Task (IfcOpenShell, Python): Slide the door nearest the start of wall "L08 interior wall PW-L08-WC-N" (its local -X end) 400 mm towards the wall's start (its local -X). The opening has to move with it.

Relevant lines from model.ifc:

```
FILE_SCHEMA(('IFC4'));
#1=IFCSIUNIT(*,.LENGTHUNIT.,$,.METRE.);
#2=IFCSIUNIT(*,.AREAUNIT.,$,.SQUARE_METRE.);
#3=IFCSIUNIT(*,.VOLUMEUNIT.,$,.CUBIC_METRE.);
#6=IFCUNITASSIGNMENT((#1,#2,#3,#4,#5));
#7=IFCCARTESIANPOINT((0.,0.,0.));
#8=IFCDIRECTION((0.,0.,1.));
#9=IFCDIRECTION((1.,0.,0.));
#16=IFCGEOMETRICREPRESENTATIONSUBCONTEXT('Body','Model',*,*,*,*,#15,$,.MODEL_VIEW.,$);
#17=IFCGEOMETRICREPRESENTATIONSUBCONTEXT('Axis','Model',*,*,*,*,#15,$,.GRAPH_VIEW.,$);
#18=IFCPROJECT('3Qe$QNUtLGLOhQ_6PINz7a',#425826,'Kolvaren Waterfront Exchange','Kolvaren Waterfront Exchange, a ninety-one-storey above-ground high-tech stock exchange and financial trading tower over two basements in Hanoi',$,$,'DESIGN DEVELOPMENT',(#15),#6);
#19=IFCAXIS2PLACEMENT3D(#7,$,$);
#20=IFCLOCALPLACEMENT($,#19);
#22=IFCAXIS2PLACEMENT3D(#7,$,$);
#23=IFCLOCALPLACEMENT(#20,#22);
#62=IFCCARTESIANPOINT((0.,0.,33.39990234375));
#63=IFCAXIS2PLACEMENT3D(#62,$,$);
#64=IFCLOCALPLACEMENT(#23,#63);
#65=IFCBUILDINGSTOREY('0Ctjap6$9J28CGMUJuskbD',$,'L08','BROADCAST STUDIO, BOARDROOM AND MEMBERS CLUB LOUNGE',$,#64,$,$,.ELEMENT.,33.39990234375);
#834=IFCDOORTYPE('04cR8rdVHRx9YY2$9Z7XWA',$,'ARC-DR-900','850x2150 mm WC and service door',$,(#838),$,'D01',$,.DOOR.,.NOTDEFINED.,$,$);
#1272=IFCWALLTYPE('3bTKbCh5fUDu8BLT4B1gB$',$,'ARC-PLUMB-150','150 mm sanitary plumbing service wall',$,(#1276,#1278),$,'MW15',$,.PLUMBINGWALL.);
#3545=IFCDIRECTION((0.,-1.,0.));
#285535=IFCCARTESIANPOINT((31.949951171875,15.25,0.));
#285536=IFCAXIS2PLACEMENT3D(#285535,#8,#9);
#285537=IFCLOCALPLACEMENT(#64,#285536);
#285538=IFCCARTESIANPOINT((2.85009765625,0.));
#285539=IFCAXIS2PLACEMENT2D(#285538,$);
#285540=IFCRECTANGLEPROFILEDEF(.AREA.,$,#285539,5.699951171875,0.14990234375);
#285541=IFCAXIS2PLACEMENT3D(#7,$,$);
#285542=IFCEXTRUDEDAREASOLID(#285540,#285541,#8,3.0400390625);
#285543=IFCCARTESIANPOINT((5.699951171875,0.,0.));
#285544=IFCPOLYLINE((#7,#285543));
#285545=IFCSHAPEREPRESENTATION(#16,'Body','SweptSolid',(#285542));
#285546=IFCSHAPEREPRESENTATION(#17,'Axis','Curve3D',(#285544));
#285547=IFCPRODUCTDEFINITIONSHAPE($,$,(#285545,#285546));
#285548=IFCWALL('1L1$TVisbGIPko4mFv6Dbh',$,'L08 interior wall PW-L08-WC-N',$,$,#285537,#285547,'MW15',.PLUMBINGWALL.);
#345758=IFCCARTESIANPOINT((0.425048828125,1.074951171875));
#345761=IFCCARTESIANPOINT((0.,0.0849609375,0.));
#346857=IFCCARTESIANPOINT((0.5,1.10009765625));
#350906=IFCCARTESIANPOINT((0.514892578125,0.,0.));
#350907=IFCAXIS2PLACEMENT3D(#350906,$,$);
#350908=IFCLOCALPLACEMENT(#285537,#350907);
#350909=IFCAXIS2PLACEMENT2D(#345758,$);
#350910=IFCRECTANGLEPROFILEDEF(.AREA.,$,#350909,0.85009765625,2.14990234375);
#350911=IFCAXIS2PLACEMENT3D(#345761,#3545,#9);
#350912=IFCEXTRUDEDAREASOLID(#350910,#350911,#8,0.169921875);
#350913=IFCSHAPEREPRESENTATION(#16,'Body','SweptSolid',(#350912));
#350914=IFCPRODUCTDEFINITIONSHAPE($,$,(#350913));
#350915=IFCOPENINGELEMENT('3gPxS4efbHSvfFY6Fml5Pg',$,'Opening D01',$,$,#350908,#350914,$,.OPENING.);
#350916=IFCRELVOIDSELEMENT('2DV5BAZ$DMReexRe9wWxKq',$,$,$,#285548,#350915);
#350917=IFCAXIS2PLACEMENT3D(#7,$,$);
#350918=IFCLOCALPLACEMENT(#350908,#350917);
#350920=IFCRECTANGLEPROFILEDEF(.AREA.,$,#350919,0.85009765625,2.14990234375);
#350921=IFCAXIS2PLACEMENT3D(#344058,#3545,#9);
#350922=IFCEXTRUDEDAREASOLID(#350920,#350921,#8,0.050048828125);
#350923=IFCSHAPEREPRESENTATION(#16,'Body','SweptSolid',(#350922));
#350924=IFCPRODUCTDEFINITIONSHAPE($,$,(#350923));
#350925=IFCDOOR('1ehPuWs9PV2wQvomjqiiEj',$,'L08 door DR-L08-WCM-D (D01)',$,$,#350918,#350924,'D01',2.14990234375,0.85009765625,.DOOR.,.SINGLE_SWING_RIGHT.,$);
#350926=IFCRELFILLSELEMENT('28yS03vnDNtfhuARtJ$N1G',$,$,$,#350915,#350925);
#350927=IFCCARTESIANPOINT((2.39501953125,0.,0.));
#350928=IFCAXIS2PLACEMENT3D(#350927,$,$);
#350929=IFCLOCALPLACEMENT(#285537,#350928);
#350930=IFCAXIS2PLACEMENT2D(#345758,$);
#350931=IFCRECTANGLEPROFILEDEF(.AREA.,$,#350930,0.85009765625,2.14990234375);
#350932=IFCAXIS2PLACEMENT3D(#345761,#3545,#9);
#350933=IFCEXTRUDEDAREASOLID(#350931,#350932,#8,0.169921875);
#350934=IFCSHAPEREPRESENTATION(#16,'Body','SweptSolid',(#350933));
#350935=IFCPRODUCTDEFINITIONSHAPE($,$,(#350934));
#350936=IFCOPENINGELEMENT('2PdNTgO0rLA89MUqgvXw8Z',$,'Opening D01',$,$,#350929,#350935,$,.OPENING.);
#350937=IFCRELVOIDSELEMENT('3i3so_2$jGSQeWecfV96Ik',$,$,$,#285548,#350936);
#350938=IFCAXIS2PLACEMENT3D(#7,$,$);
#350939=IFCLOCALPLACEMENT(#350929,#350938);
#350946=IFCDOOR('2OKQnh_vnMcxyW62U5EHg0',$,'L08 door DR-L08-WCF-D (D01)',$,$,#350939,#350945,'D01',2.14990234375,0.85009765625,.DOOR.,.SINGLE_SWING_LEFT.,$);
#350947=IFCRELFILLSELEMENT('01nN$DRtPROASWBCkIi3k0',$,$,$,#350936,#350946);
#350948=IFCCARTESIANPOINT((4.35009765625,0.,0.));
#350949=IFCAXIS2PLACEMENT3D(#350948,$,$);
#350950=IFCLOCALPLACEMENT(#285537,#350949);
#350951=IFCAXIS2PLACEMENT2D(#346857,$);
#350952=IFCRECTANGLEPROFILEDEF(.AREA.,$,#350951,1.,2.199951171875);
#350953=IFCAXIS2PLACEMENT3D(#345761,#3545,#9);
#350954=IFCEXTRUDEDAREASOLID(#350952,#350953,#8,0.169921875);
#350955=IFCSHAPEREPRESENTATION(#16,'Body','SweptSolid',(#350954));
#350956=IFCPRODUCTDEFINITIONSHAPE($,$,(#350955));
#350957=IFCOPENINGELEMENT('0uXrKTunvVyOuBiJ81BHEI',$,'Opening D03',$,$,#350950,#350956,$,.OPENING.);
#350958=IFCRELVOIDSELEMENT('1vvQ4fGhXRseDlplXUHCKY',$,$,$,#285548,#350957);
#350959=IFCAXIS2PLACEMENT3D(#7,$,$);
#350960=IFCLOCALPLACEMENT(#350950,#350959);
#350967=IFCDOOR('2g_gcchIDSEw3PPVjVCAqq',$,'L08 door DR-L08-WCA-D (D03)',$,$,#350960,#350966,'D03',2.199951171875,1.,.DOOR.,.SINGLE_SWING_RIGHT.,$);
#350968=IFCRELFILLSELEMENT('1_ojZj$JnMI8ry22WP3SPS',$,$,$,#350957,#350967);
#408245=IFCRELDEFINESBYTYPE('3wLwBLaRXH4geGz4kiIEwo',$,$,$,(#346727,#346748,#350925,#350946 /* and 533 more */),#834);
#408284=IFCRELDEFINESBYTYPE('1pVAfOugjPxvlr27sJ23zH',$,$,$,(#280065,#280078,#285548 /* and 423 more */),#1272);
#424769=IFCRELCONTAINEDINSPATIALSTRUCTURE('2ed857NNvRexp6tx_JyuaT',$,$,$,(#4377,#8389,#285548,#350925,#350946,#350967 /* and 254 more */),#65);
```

```python
import ifcopenshell
import ifcopenshell.api.geometry
import ifcopenshell.util.placement
import ifcopenshell.util.unit

model = ifcopenshell.open("model.ifc")
unit_scale = ifcopenshell.util.unit.calculate_unit_scale(model)

door = model.by_guid("1ehPuWs9PV2wQvomjqiiEj")
opening = door.FillsVoids[0].RelatingOpeningElement
wall = opening.VoidsElements[0].RelatingBuildingElement

wall_matrix = ifcopenshell.util.placement.get_local_placement(wall.ObjectPlacement)
shift = wall_matrix[:3, 0] * -0.4 / unit_scale
before = ifcopenshell.util.placement.get_local_placement(door.ObjectPlacement)[:3, 3].copy()

# The door is placed relative to its opening, so it follows when the opening moves.
matrix = ifcopenshell.util.placement.get_local_placement(opening.ObjectPlacement)
matrix[:3, 3] += shift
ifcopenshell.api.geometry.edit_object_placement(
    model, product=opening, matrix=matrix, is_si=False, should_transform_children=True
)

after = ifcopenshell.util.placement.get_local_placement(door.ObjectPlacement)[:3, 3]
print("door moved by", (after - before).round(3) + 0.0)

model.write("model_edited.ifc")
```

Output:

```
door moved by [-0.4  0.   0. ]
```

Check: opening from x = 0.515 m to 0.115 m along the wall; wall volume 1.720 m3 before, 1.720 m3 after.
